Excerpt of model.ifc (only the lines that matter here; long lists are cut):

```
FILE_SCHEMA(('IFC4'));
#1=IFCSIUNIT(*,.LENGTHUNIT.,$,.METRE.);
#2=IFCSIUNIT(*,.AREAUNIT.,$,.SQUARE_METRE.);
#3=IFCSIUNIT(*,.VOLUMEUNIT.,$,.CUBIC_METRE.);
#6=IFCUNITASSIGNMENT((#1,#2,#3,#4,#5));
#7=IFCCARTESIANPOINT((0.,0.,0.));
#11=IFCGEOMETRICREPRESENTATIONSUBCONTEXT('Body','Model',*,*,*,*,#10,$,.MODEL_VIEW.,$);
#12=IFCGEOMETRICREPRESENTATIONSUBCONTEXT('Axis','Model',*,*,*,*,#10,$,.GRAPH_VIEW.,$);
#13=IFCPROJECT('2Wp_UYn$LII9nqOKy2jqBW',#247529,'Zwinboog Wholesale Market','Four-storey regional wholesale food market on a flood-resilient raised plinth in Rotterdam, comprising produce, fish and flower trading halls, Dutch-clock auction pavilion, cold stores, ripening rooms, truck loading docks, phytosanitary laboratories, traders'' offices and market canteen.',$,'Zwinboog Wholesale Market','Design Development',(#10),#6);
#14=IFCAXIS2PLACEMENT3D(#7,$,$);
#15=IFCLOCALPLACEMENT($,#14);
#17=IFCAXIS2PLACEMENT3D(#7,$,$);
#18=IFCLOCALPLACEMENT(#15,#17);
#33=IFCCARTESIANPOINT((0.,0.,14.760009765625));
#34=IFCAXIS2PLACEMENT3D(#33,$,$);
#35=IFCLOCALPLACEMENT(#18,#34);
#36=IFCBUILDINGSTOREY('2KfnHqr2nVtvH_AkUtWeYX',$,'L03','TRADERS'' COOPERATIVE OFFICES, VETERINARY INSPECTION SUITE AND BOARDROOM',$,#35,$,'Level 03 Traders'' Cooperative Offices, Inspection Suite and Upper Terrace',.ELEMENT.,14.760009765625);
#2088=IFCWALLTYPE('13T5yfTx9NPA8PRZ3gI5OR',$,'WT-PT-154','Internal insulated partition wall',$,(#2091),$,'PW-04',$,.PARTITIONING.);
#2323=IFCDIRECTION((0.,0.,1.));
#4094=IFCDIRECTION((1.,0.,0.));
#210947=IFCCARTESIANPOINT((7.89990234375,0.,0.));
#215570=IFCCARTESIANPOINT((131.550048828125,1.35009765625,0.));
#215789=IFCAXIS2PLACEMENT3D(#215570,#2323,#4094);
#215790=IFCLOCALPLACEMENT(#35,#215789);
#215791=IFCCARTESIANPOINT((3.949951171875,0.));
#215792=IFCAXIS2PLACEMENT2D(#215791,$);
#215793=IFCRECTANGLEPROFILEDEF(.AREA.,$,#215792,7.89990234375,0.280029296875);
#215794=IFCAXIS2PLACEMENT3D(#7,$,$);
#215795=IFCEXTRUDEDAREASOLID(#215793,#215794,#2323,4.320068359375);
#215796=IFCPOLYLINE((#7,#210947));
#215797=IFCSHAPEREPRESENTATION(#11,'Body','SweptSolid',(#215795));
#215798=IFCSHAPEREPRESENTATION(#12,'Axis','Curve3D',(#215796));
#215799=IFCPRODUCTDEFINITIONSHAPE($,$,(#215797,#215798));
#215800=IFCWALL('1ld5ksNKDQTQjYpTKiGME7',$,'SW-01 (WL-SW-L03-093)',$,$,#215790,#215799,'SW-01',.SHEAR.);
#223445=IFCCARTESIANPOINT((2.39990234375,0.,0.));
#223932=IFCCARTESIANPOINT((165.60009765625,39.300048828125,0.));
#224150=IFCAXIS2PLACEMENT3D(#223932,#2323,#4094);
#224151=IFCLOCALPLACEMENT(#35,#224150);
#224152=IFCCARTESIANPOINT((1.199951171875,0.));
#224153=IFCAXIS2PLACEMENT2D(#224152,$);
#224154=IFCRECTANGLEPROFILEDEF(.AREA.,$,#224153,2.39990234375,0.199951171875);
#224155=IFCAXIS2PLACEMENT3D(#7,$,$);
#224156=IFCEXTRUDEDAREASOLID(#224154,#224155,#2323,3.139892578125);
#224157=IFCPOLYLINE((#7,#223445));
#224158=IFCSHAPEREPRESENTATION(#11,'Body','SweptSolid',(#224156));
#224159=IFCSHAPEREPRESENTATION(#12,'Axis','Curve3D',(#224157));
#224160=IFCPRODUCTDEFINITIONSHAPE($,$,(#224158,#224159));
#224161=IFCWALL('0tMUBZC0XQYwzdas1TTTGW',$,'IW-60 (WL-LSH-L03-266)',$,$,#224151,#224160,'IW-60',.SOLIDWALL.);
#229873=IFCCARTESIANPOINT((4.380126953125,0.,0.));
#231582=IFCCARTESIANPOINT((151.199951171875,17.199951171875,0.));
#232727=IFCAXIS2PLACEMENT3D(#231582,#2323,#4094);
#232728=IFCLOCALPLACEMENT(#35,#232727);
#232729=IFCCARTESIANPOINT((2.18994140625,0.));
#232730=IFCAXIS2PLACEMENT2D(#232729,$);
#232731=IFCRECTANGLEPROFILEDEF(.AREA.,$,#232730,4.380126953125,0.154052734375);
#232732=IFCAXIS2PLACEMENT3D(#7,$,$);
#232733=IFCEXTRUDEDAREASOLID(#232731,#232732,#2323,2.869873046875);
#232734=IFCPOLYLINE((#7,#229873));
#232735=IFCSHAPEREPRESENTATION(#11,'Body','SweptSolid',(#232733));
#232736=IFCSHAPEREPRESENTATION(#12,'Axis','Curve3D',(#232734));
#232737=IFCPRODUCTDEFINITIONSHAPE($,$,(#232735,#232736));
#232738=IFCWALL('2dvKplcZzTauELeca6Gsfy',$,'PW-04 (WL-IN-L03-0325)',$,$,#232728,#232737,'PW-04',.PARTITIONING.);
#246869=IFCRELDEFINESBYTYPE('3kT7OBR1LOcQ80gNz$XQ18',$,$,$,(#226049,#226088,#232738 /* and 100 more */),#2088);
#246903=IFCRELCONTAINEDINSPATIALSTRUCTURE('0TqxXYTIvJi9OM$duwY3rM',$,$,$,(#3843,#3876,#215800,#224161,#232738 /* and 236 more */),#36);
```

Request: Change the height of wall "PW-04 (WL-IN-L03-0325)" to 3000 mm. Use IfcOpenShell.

```python
import ifcopenshell
import ifcopenshell.geom
import ifcopenshell.util.representation
import ifcopenshell.util.shape

model = ifcopenshell.open("model.ifc")
settings = ifcopenshell.geom.settings()


def volume(element):
    """Net volume in cubic metres, openings subtracted."""
    shape = ifcopenshell.geom.create_shape(settings, element)
    return ifcopenshell.util.shape.get_volume(shape.geometry)


wall = model.by_guid("2dvKplcZzTauELeca6Gsfy")
before = volume(wall)

body = ifcopenshell.util.representation.get_representation(wall, "Model", "Body")
solid = body.Items[0]
old_height = solid.Depth
solid.Depth = 3.0
after = volume(wall)

print(f"height {old_height:g} -> {solid.Depth:g}, volume {before:.3f} -> {after:.3f} m3")

model.write("model_v2.ifc")
```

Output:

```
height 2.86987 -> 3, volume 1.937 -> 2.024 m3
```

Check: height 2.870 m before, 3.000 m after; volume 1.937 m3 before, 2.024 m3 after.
